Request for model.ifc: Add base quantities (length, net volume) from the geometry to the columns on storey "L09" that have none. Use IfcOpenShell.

First a look at what the model holds.

```python
import ifcopenshell
import ifcopenshell.util.element
import ifcopenshell.util.unit

model = ifcopenshell.open("model.ifc")
print(model.schema)
for unit_type in ("LENGTHUNIT", "AREAUNIT", "VOLUMEUNIT"):
    print(unit_type, ifcopenshell.util.unit.calculate_unit_scale(model, unit_type))
storey = next(s for s in model.by_type("IfcBuildingStorey") if s.Name == "L09")
columns = [e for e in ifcopenshell.util.element.get_decomposition(storey) if e.is_a("IfcColumn")]
for e in sorted(columns, key=lambda e: e.id()):
    print(e.id(), e.is_a(), e.Name, list(ifcopenshell.util.element.get_psets(e, qtos_only=True)), sep=" | ")
```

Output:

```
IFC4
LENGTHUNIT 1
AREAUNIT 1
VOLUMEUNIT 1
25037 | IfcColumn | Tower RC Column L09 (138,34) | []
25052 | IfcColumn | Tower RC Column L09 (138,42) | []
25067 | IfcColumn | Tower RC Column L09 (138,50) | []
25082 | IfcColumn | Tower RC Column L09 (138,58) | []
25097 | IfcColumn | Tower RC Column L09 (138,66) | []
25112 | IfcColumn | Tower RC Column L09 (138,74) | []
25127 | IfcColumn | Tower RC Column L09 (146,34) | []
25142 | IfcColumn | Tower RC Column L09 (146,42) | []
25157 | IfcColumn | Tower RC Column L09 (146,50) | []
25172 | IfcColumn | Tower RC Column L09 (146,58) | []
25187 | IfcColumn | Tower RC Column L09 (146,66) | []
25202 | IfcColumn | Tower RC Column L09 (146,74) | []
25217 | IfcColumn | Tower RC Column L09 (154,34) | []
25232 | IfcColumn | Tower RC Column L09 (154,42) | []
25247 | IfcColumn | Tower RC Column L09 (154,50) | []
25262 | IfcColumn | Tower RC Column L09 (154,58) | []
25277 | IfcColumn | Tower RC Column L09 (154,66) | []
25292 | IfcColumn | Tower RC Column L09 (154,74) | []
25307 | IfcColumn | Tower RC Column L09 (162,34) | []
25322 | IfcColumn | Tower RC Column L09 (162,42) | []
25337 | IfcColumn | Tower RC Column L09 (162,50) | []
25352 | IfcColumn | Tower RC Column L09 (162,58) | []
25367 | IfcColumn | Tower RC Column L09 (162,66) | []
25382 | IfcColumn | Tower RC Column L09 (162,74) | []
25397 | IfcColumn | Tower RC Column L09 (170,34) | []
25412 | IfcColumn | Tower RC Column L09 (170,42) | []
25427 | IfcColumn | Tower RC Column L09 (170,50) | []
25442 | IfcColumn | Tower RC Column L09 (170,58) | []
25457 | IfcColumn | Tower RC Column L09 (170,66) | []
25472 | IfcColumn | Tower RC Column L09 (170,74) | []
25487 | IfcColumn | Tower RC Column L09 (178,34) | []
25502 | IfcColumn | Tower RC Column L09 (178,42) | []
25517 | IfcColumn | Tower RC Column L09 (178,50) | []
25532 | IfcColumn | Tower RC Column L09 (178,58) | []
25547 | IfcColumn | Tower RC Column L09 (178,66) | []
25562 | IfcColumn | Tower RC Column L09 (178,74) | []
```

```python
import ifcopenshell
import ifcopenshell.api.pset
import ifcopenshell.geom
import ifcopenshell.util.element
import ifcopenshell.util.shape
import ifcopenshell.util.unit

model = ifcopenshell.open("model.ifc")
unit_scale = ifcopenshell.util.unit.calculate_unit_scale(model)
volume_scale = ifcopenshell.util.unit.calculate_unit_scale(model, "VOLUMEUNIT")
settings = ifcopenshell.geom.settings()

storey = next(s for s in model.by_type("IfcBuildingStorey") if s.Name == "L09")
columns = [e for e in ifcopenshell.util.element.get_decomposition(storey) if e.is_a("IfcColumn")]

for e in sorted(columns, key=lambda e: e.id()):
    if ifcopenshell.util.element.get_psets(e, qtos_only=True, should_inherit=False):
        continue
    # Geometry comes back in metres, in the element's own axes.
    shape = ifcopenshell.geom.create_shape(settings, e)
    values = {
        "Length": ifcopenshell.util.shape.get_z(shape.geometry) / unit_scale,
        "NetVolume": ifcopenshell.util.shape.get_volume(shape.geometry) / volume_scale,
    }
    qto = ifcopenshell.api.pset.add_qto(model, product=e, name="Qto_ColumnBaseQuantities")
    ifcopenshell.api.pset.edit_qto(model, qto=qto, properties=values)
    print(e.id(), {k: round(v, 3) for k, v in values.items()})

model.write("model_edited.ifc")
```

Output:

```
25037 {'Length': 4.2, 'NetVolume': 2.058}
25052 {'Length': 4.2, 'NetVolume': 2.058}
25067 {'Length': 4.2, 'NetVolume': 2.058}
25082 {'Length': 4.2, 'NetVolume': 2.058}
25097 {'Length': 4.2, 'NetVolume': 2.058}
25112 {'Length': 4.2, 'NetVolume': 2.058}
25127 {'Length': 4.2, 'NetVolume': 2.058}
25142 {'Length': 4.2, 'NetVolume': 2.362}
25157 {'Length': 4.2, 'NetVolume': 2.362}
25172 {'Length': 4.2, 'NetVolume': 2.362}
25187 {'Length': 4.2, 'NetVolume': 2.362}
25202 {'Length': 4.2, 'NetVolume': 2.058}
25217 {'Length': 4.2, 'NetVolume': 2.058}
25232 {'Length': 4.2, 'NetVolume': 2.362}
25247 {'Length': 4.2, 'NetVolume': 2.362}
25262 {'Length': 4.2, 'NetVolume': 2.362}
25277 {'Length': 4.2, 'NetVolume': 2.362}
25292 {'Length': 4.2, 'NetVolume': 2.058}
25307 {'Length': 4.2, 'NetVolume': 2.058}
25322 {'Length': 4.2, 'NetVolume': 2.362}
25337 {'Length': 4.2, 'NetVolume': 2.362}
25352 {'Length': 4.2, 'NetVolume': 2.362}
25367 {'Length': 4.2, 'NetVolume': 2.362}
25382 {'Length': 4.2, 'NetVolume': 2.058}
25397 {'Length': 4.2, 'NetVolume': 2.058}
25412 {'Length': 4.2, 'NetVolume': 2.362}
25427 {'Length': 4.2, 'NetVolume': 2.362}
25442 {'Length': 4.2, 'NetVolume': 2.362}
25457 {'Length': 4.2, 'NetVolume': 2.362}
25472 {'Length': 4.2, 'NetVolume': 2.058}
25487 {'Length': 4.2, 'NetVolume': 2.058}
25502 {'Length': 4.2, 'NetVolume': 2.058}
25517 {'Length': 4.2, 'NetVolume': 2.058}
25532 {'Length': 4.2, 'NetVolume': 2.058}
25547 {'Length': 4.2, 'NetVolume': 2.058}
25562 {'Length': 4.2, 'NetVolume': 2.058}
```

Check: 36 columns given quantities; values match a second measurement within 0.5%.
